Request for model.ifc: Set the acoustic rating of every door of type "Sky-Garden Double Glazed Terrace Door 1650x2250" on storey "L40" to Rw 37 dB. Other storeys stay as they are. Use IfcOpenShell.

First a look at what the model holds.

```python
import ifcopenshell
import ifcopenshell.util.element

model = ifcopenshell.open("model.ifc")
print(model.schema)
storey = next(s for s in model.by_type("IfcBuildingStorey") if s.Name == "L40")
doors = [e for e in ifcopenshell.util.element.get_decomposition(storey) if e.is_a("IfcDoor")]
seen = {}
for e in doors:
    element_type = ifcopenshell.util.element.get_type(e)
    key = (element_type.Name if element_type != e and element_type else None, ifcopenshell.util.element.get_pset(e, "Pset_DoorCommon", "AcousticRating"))
    seen[key] = seen.get(key, 0) + 1
for (name, value), count in sorted(seen.items(), key=str):
    print(count, "x", name, "|", value)
```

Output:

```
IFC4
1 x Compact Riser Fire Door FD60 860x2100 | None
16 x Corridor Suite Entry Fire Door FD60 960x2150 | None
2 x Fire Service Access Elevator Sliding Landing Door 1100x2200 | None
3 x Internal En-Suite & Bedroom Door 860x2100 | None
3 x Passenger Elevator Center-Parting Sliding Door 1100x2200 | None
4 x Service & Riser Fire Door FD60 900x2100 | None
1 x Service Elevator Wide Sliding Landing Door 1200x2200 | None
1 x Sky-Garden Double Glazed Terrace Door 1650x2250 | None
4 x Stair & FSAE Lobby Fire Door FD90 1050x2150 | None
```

```python
import ifcopenshell
import ifcopenshell.api.pset
import ifcopenshell.util.element

model = ifcopenshell.open("model.ifc")

storey = next(s for s in model.by_type("IfcBuildingStorey") if s.Name == "L40")
doors = [e for e in ifcopenshell.util.element.get_decomposition(storey) if e.is_a("IfcDoor")]

count = 0
for e in doors:
    element_type = ifcopenshell.util.element.get_type(e)
    if element_type in (None, e) or element_type.Name != "Sky-Garden Double Glazed Terrace Door 1650x2250":
        continue
    found = ifcopenshell.util.element.get_pset(e, "Pset_DoorCommon", should_inherit=False)
    if found:
        pset = model.by_id(found["id"])
        if len(ifcopenshell.util.element.get_elements_by_pset(pset)) > 1:
            pset = ifcopenshell.api.pset.unshare_pset(model, products=[e], pset=pset)[0]
    else:
        pset = ifcopenshell.api.pset.add_pset(model, product=e, name="Pset_DoorCommon")
    ifcopenshell.api.pset.edit_pset(model, pset=pset, properties={"AcousticRating": "Rw 37 dB"})
    count += 1

print(count, "doors updated")

model.write("model_updated.ifc")
```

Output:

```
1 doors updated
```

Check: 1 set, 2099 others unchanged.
